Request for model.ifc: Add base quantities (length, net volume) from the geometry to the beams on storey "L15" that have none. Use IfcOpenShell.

First a look at what the model holds.

```python
import ifcopenshell
import ifcopenshell.util.element
import ifcopenshell.util.unit

model = ifcopenshell.open("model.ifc")
print(model.schema)
for unit_type in ("LENGTHUNIT", "AREAUNIT", "VOLUMEUNIT"):
    print(unit_type, ifcopenshell.util.unit.calculate_unit_scale(model, unit_type))
storey = next(s for s in model.by_type("IfcBuildingStorey") if s.Name == "L15")
beams = [e for e in ifcopenshell.util.element.get_decomposition(storey) if e.is_a("IfcBeam")]
for e in sorted(beams, key=lambda e: e.id()):
    print(e.id(), e.is_a(), e.Name, list(ifcopenshell.util.element.get_psets(e, qtos_only=True)), sep=" | ")
```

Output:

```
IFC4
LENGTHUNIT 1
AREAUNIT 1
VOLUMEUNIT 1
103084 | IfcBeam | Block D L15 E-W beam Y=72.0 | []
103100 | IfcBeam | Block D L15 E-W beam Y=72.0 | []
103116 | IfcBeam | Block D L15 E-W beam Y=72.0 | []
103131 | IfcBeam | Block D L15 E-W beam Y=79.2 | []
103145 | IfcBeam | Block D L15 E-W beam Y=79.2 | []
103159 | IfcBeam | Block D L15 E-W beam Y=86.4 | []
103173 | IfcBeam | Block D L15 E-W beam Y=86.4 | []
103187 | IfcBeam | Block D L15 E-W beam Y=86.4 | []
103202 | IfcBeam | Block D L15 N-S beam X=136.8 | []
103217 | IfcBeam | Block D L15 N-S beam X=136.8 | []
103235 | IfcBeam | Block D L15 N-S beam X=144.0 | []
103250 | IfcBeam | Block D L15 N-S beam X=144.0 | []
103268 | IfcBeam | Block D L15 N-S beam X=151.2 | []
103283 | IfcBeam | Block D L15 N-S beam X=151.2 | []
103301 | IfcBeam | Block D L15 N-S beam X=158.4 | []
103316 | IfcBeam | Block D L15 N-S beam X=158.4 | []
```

```python
import ifcopenshell
import ifcopenshell.api.pset
import ifcopenshell.geom
import ifcopenshell.util.element
import ifcopenshell.util.shape
import ifcopenshell.util.unit

model = ifcopenshell.open("model.ifc")
unit_scale = ifcopenshell.util.unit.calculate_unit_scale(model)
volume_scale = ifcopenshell.util.unit.calculate_unit_scale(model, "VOLUMEUNIT")
settings = ifcopenshell.geom.settings()

storey = next(s for s in model.by_type("IfcBuildingStorey") if s.Name == "L15")
beams = [e for e in ifcopenshell.util.element.get_decomposition(storey) if e.is_a("IfcBeam")]

for e in sorted(beams, key=lambda e: e.id()):
    if ifcopenshell.util.element.get_psets(e, qtos_only=True, should_inherit=False):
        continue
    # Geometry comes back in metres, in the element's own axes.
    shape = ifcopenshell.geom.create_shape(settings, e)
    values = {
        "Length": ifcopenshell.util.shape.get_max_xyz(shape.geometry) / unit_scale,
        "NetVolume": ifcopenshell.util.shape.get_volume(shape.geometry) / volume_scale,
    }
    qto = ifcopenshell.api.pset.add_qto(model, product=e, name="Qto_BeamBaseQuantities")
    ifcopenshell.api.pset.edit_qto(model, qto=qto, properties=values)
    print(e.id(), {k: round(v, 3) for k, v in values.items()})

model.write("model_edited.ifc")
```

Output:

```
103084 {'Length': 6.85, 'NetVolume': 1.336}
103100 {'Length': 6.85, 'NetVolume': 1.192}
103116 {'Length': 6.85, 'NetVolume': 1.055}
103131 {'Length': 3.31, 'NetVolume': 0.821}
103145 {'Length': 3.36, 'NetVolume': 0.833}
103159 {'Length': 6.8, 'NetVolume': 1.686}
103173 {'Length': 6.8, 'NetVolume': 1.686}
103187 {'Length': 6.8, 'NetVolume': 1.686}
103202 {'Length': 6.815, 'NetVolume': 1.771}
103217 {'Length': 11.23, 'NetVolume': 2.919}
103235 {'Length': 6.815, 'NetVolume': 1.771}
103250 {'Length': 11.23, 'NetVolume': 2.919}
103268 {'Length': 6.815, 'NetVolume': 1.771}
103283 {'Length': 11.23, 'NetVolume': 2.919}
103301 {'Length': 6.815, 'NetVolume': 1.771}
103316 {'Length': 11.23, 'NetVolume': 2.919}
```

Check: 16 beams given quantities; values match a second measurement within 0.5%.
